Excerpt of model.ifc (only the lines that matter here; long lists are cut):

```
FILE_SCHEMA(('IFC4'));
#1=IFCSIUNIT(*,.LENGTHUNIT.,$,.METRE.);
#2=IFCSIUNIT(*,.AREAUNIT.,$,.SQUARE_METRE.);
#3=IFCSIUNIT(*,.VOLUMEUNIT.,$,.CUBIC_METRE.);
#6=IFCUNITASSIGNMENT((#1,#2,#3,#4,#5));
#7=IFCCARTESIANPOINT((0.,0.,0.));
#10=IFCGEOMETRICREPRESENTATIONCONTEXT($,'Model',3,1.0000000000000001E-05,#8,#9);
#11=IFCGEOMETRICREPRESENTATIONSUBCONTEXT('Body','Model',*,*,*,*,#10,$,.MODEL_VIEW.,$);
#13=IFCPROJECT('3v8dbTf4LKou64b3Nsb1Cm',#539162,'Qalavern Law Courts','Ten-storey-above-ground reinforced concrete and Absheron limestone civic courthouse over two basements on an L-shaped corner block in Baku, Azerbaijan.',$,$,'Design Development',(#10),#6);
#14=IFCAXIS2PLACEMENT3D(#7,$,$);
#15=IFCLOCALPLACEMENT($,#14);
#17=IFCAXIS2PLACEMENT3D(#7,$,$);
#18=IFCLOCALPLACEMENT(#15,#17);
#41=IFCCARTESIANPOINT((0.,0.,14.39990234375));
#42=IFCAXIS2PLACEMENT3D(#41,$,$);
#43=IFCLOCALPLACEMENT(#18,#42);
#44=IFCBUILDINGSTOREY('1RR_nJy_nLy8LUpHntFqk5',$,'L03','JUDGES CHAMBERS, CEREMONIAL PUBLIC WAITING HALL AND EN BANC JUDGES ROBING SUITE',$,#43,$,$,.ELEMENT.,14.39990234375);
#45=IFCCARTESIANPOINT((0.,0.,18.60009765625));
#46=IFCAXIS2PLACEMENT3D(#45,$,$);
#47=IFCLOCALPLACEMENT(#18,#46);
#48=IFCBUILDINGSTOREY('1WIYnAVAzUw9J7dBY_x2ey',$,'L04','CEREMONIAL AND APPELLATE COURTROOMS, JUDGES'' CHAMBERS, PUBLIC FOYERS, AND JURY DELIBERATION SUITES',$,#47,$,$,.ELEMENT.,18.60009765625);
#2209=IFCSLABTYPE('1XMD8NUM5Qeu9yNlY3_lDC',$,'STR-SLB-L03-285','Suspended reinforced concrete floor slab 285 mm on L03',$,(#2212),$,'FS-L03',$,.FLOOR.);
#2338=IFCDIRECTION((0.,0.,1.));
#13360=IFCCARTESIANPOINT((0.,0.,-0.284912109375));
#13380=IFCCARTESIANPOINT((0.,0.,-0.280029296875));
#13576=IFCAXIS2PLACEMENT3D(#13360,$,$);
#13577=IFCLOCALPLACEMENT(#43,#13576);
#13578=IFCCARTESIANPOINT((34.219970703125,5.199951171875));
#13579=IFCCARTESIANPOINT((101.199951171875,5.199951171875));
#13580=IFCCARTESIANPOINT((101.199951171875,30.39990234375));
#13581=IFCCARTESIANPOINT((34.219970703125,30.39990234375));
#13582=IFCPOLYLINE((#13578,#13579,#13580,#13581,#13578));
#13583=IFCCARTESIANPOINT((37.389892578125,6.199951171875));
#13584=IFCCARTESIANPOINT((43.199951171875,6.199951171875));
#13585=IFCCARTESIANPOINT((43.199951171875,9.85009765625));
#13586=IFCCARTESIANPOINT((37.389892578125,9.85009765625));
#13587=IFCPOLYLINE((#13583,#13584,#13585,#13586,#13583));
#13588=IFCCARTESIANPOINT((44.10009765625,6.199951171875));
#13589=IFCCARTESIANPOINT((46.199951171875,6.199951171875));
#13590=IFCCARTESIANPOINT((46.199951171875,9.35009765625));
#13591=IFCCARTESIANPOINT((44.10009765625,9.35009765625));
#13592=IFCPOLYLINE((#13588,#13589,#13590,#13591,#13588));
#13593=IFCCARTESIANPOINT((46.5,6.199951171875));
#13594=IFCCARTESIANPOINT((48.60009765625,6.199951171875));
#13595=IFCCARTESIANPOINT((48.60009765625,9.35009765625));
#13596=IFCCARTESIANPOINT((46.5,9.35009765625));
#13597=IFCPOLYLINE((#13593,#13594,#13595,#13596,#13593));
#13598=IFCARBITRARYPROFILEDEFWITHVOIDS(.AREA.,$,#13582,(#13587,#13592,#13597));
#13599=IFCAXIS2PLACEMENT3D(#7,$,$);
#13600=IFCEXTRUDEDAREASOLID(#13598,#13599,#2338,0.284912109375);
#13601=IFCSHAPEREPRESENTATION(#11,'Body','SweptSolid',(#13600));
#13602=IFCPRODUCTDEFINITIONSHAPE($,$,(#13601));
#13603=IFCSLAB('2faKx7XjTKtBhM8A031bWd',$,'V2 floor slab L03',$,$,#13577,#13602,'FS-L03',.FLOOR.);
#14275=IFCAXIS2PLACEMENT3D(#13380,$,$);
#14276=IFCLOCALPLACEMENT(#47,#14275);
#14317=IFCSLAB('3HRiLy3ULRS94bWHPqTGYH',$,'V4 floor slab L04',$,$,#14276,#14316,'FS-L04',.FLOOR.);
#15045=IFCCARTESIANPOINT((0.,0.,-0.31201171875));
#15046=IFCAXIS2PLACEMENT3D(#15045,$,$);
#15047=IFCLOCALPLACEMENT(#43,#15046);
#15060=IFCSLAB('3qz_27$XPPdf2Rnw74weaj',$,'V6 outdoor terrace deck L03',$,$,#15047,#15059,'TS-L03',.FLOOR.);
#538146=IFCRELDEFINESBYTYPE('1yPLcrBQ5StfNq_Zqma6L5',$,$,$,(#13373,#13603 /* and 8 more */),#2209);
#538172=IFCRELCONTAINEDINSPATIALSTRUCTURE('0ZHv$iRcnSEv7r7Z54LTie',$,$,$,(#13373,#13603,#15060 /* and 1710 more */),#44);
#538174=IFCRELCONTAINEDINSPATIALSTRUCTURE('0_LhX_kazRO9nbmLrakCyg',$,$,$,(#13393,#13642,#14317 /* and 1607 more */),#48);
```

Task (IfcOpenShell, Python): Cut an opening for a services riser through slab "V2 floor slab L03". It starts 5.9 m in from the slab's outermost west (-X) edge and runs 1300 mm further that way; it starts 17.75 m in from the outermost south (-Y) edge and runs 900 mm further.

```python
import numpy as np
import ifcopenshell
import ifcopenshell.api.feature
import ifcopenshell.api.geometry
import ifcopenshell.api.root
import ifcopenshell.geom
import ifcopenshell.util.placement
import ifcopenshell.util.representation
import ifcopenshell.util.shape
import ifcopenshell.util.unit

model = ifcopenshell.open("model.ifc")
unit_scale = ifcopenshell.util.unit.calculate_unit_scale(model)
settings = ifcopenshell.geom.settings()


def volume(element):
    """Net volume in cubic metres, openings subtracted."""
    shape = ifcopenshell.geom.create_shape(settings, element)
    return ifcopenshell.util.shape.get_volume(shape.geometry)


slab = model.by_guid("2faKx7XjTKtBhM8A031bWd")
before = volume(slab)

# Extent in the slab's own axes, in metres. The edges named are its -X and -Y sides.
slab_shape = ifcopenshell.geom.create_shape(settings, slab)
vertices = ifcopenshell.util.shape.get_vertices(slab_shape.geometry)
x_min, y_min, bottom = vertices.min(axis=0)
top = vertices[:, 2].max()

opening = ifcopenshell.api.root.create_entity(model, ifc_class="IfcOpeningElement", name="Services riser opening", predefined_type="OPENING")
context = ifcopenshell.util.representation.get_context(model, "Model", "Body", "MODEL_VIEW")
width, depth = 1.3, 0.9
outline = [(0.0, 0.0), (width, 0.0), (width, depth), (0.0, depth), (0.0, 0.0)]
# Overshoot both faces by 50 mm so the cut is clean.
shape = ifcopenshell.api.geometry.add_slab_representation(
    model, context=context, depth=top - bottom + 0.1, polyline=outline
)
ifcopenshell.api.geometry.assign_representation(model, product=opening, representation=shape)

matrix = ifcopenshell.util.placement.get_local_placement(slab.ObjectPlacement)
matrix[:, 3] = matrix @ np.append(np.array([x_min + 5.9, y_min + 17.75, bottom - 0.05]) / unit_scale, 1.0)
ifcopenshell.api.geometry.edit_object_placement(model, product=opening, matrix=matrix, is_si=False)
ifcopenshell.api.feature.add_feature(model, feature=opening, element=slab)

after = volume(slab)

print(f"slab volume {before:.3f} -> {after:.3f} m3")

model.write("model_edited.ifc")
```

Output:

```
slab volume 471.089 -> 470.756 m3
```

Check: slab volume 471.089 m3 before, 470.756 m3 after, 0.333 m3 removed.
